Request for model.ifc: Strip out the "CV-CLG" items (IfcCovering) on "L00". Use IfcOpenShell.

First a look at what the model holds.

```python
import ifcopenshell
import ifcopenshell.util.element

model = ifcopenshell.open("model.ifc")
print(model.schema)
storey = next(s for s in model.by_type("IfcBuildingStorey") if s.Name == "L00")
coverings = [e for e in ifcopenshell.util.element.get_decomposition(storey) if e.is_a("IfcCovering")]
seen = {}
for e in coverings:
    element_type = ifcopenshell.util.element.get_type(e)
    name = element_type.Name if element_type not in (None, e) else None
    seen[name] = seen.get(name, 0) + 1
for name, count in sorted(seen.items(), key=str):
    print(count, "x", name)
```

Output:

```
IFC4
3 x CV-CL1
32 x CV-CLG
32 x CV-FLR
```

```python
import ifcopenshell
import ifcopenshell.api.root
import ifcopenshell.util.element

model = ifcopenshell.open("model.ifc")

storey = next(s for s in model.by_type("IfcBuildingStorey") if s.Name == "L00")
coverings = [e for e in ifcopenshell.util.element.get_decomposition(storey) if e.is_a("IfcCovering")]
targets = [e for e in coverings if (t := ifcopenshell.util.element.get_type(e)) not in (None, e) and t.Name == "CV-CLG"]

for e in targets:
    ifcopenshell.api.root.remove_product(model, product=e)
print(len(targets), "removed")

model.write("model_updated.ifc")
```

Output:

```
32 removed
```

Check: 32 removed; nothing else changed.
